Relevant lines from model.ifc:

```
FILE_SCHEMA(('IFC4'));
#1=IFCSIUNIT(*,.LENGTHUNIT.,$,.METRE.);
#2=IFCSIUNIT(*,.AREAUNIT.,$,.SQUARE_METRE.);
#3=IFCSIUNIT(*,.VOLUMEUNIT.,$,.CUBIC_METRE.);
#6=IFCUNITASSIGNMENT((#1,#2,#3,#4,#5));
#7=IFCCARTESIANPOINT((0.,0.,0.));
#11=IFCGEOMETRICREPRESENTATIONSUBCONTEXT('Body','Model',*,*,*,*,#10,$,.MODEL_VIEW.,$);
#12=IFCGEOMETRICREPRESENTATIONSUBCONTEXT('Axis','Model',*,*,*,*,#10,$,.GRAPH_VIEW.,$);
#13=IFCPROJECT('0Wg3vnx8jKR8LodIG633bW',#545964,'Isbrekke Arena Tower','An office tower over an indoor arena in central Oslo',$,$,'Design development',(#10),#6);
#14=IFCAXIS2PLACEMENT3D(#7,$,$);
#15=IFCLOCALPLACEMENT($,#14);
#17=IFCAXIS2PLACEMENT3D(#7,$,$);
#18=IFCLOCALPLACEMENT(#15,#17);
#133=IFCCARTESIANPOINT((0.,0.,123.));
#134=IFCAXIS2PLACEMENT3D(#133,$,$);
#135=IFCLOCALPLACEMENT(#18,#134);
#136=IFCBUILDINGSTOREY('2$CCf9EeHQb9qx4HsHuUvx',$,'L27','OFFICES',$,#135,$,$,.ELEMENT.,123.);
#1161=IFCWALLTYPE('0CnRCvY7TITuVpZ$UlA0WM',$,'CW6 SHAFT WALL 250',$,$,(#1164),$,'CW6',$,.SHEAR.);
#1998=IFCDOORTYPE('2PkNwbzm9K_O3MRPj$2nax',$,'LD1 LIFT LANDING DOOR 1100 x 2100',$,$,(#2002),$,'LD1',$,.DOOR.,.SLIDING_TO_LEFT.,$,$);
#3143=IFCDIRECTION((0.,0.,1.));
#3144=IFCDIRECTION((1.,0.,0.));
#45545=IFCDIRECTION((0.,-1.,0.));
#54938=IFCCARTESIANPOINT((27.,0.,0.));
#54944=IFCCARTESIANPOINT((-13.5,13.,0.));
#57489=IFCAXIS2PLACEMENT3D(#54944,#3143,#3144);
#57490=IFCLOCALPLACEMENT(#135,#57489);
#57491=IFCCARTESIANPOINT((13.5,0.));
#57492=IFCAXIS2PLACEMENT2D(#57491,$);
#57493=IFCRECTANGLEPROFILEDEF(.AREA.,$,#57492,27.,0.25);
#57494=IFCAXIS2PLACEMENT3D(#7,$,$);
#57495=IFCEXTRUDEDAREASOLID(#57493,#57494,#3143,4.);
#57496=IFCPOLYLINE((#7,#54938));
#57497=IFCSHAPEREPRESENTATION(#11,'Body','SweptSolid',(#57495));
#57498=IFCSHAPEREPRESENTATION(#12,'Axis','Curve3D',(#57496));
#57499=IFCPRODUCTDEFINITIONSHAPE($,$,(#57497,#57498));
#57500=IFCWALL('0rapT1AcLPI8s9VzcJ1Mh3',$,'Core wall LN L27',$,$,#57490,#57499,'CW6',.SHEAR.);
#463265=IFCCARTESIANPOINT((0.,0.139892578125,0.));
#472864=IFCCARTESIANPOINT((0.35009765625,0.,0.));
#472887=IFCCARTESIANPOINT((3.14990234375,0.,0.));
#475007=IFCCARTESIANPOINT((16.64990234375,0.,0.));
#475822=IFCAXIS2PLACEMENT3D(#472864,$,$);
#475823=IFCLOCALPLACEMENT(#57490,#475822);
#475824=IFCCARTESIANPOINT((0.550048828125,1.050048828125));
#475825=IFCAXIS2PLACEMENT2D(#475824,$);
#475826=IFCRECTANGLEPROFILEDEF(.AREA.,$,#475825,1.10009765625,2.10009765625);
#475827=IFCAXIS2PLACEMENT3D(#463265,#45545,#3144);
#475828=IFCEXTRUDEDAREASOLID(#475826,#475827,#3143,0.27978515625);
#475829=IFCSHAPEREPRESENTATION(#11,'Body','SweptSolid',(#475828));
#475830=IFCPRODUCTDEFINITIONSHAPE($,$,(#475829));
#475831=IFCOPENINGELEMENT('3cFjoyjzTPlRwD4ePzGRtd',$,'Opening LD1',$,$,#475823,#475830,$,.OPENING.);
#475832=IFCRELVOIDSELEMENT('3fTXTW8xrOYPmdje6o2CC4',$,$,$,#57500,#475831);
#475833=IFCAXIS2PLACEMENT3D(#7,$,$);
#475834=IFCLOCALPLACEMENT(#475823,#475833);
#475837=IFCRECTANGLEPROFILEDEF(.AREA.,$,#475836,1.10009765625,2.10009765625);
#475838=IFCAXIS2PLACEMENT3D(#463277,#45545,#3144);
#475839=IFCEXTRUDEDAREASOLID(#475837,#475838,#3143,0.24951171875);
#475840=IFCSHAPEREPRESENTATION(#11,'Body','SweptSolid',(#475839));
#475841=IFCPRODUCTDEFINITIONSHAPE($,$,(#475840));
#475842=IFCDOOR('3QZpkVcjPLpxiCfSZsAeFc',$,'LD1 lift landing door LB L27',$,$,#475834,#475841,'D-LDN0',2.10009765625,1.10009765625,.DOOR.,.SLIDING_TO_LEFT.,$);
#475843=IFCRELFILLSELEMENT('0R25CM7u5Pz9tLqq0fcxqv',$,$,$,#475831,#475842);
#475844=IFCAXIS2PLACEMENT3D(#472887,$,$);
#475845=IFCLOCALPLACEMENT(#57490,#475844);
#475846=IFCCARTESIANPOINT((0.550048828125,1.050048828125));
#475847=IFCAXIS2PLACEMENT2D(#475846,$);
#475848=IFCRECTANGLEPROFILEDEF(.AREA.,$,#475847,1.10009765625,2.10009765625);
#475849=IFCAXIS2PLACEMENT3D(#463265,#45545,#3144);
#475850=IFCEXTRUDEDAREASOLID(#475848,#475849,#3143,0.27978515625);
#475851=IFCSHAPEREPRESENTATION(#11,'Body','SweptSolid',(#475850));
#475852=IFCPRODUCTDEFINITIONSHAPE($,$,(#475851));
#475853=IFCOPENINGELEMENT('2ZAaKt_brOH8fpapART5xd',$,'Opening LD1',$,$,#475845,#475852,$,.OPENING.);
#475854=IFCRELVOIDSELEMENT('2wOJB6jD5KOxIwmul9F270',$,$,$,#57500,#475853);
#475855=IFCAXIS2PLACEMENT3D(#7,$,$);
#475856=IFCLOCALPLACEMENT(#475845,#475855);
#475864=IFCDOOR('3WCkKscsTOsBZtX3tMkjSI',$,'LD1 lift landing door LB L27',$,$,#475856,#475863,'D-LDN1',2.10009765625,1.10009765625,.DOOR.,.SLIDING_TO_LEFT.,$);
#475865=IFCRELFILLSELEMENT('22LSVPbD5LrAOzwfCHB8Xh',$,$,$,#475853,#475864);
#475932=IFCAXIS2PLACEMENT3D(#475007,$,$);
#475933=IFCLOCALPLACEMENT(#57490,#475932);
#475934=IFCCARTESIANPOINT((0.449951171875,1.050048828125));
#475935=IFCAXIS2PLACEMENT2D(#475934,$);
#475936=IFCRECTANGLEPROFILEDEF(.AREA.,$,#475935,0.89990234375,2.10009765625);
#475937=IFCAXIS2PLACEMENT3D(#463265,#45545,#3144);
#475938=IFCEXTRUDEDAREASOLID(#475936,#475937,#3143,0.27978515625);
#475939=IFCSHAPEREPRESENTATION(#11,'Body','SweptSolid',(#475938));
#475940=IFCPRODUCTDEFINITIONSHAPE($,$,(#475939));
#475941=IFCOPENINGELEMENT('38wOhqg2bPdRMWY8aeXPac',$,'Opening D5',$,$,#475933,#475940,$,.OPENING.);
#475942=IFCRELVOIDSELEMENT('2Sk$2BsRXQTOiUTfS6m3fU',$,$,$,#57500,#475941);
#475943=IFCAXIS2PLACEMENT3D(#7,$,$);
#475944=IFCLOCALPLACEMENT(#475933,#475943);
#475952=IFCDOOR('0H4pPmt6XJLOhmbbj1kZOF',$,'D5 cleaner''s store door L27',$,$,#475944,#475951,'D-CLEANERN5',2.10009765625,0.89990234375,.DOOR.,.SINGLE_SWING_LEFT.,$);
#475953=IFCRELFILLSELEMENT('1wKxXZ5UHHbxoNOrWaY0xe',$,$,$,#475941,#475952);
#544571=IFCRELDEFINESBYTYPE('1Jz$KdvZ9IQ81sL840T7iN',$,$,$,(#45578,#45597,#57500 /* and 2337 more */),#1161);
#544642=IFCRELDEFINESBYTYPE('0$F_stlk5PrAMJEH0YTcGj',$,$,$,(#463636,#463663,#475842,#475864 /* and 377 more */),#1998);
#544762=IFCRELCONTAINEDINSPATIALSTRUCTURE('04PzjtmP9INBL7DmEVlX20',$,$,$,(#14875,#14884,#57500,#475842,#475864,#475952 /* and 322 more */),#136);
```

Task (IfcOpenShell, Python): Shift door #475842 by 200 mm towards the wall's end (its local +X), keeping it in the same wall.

```python
import ifcopenshell
import ifcopenshell.api.geometry
import ifcopenshell.util.placement

model = ifcopenshell.open("model.ifc")

door = model.by_id(475842)
opening = door.FillsVoids[0].RelatingOpeningElement
wall = opening.VoidsElements[0].RelatingBuildingElement

wall_matrix = ifcopenshell.util.placement.get_local_placement(wall.ObjectPlacement)
shift = wall_matrix[:3, 0] * 0.2
before = ifcopenshell.util.placement.get_local_placement(door.ObjectPlacement)[:3, 3].copy()

# The door is placed relative to its opening, so it follows when the opening moves.
matrix = ifcopenshell.util.placement.get_local_placement(opening.ObjectPlacement)
matrix[:3, 3] += shift
ifcopenshell.api.geometry.edit_object_placement(
    model, product=opening, matrix=matrix, is_si=False, should_transform_children=True
)

after = ifcopenshell.util.placement.get_local_placement(door.ObjectPlacement)[:3, 3]
print("door moved by", (after - before).round(3) + 0.0)

model.write("model_rev.ifc")
```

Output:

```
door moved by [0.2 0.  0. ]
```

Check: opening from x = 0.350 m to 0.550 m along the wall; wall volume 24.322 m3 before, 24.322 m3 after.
